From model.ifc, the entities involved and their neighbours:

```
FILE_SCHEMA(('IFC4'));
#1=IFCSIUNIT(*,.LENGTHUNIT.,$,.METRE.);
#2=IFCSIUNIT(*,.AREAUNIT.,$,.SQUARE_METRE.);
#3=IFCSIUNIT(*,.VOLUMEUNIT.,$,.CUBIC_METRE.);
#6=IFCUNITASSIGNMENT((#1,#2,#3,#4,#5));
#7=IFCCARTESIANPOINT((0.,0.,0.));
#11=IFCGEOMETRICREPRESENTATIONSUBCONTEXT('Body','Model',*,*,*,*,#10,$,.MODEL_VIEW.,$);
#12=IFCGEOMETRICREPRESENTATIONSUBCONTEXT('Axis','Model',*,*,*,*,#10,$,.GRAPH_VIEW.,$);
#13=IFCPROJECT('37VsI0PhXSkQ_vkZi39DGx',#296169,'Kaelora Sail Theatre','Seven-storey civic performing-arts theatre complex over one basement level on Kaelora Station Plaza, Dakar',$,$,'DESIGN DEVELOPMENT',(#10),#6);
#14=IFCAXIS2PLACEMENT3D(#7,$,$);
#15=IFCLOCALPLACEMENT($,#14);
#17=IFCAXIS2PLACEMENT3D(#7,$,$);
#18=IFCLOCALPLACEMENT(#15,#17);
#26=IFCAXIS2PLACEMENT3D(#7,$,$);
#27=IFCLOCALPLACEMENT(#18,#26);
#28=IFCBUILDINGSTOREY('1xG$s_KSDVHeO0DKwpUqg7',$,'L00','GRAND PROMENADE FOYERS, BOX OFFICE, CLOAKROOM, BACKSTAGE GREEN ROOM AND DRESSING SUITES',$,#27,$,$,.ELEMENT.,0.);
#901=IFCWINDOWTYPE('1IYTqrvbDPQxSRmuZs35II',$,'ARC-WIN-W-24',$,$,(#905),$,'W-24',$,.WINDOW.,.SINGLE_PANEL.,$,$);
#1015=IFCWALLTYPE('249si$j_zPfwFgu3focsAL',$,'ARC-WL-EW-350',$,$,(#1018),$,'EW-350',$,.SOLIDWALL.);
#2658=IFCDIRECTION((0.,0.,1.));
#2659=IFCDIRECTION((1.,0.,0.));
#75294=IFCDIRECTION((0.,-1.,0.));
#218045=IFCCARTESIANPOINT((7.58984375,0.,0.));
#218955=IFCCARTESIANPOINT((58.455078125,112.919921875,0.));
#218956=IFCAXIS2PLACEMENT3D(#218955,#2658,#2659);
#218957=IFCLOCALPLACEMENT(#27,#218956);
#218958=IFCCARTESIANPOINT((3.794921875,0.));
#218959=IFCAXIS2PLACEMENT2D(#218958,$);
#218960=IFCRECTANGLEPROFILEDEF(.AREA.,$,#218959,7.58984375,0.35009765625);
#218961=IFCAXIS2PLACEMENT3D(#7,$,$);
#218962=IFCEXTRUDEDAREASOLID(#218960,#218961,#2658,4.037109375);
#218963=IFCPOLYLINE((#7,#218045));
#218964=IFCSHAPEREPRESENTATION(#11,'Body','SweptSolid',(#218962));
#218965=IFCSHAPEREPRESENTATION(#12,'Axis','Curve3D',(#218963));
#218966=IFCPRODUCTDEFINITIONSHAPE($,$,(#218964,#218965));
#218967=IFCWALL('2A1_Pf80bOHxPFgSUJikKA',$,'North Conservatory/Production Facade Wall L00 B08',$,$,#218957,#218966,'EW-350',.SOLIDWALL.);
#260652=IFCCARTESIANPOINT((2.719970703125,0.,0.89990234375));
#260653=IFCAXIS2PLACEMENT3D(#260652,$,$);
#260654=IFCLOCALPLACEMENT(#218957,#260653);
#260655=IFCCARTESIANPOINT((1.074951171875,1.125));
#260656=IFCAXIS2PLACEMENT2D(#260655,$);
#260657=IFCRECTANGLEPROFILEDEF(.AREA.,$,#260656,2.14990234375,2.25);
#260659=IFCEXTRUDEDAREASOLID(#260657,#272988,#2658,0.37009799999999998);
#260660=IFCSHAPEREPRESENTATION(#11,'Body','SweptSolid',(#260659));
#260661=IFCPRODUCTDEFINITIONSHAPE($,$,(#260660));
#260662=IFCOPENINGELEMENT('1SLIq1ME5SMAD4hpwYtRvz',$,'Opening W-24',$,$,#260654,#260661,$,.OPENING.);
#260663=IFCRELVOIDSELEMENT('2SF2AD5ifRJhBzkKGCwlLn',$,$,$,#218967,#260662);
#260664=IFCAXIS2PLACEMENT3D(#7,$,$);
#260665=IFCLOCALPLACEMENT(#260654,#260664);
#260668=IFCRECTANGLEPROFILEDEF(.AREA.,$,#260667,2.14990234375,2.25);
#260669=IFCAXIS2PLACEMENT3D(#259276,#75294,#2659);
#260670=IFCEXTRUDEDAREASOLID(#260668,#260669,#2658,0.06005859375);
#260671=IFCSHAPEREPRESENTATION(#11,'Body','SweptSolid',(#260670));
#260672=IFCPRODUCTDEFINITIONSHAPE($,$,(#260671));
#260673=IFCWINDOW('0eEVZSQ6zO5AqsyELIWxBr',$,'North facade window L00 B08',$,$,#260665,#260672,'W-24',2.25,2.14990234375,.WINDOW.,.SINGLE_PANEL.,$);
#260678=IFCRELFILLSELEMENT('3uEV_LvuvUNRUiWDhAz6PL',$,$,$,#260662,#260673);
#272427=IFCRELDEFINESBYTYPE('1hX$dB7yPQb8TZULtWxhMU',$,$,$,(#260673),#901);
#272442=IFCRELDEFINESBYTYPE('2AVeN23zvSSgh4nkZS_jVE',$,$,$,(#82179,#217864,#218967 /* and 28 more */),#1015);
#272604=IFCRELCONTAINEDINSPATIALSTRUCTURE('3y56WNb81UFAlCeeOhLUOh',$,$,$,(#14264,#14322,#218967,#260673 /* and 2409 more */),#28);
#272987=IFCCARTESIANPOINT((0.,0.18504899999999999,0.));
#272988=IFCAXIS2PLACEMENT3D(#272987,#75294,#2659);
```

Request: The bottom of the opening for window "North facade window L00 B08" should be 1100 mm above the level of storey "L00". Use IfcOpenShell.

```python
import numpy as np
import ifcopenshell
import ifcopenshell.api.geometry
import ifcopenshell.geom
import ifcopenshell.util.element
import ifcopenshell.util.placement
import ifcopenshell.util.shape
import ifcopenshell.util.unit

model = ifcopenshell.open("model.ifc")
unit_scale = ifcopenshell.util.unit.calculate_unit_scale(model)

window = model.by_id(260673)
opening = window.FillsVoids[0].RelatingOpeningElement
storey = ifcopenshell.util.element.get_container(window, ifc_class="IfcBuildingStorey")
level = ifcopenshell.util.placement.get_local_placement(storey.ObjectPlacement)[2, 3]

# The opening's origin need not be at the sill, so measure its lowest point.
shape = ifcopenshell.geom.create_shape(ifcopenshell.geom.settings(), opening)
bottom = ifcopenshell.util.shape.get_shape_bottom_elevation(shape, shape.geometry) / unit_scale
dz = level + 1.1 - bottom

shift = np.array([0.0, 0.0, dz])
# The window is placed relative to its opening, so it follows when the opening moves.
matrix = ifcopenshell.util.placement.get_local_placement(opening.ObjectPlacement)
matrix[:3, 3] += shift
ifcopenshell.api.geometry.edit_object_placement(
    model, product=opening, matrix=matrix, is_si=False, should_transform_children=True
)

print(f"moved by {dz * unit_scale:+.3f} m")

model.write("model_rev.ifc")
```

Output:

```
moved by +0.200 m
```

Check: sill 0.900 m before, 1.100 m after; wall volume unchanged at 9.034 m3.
